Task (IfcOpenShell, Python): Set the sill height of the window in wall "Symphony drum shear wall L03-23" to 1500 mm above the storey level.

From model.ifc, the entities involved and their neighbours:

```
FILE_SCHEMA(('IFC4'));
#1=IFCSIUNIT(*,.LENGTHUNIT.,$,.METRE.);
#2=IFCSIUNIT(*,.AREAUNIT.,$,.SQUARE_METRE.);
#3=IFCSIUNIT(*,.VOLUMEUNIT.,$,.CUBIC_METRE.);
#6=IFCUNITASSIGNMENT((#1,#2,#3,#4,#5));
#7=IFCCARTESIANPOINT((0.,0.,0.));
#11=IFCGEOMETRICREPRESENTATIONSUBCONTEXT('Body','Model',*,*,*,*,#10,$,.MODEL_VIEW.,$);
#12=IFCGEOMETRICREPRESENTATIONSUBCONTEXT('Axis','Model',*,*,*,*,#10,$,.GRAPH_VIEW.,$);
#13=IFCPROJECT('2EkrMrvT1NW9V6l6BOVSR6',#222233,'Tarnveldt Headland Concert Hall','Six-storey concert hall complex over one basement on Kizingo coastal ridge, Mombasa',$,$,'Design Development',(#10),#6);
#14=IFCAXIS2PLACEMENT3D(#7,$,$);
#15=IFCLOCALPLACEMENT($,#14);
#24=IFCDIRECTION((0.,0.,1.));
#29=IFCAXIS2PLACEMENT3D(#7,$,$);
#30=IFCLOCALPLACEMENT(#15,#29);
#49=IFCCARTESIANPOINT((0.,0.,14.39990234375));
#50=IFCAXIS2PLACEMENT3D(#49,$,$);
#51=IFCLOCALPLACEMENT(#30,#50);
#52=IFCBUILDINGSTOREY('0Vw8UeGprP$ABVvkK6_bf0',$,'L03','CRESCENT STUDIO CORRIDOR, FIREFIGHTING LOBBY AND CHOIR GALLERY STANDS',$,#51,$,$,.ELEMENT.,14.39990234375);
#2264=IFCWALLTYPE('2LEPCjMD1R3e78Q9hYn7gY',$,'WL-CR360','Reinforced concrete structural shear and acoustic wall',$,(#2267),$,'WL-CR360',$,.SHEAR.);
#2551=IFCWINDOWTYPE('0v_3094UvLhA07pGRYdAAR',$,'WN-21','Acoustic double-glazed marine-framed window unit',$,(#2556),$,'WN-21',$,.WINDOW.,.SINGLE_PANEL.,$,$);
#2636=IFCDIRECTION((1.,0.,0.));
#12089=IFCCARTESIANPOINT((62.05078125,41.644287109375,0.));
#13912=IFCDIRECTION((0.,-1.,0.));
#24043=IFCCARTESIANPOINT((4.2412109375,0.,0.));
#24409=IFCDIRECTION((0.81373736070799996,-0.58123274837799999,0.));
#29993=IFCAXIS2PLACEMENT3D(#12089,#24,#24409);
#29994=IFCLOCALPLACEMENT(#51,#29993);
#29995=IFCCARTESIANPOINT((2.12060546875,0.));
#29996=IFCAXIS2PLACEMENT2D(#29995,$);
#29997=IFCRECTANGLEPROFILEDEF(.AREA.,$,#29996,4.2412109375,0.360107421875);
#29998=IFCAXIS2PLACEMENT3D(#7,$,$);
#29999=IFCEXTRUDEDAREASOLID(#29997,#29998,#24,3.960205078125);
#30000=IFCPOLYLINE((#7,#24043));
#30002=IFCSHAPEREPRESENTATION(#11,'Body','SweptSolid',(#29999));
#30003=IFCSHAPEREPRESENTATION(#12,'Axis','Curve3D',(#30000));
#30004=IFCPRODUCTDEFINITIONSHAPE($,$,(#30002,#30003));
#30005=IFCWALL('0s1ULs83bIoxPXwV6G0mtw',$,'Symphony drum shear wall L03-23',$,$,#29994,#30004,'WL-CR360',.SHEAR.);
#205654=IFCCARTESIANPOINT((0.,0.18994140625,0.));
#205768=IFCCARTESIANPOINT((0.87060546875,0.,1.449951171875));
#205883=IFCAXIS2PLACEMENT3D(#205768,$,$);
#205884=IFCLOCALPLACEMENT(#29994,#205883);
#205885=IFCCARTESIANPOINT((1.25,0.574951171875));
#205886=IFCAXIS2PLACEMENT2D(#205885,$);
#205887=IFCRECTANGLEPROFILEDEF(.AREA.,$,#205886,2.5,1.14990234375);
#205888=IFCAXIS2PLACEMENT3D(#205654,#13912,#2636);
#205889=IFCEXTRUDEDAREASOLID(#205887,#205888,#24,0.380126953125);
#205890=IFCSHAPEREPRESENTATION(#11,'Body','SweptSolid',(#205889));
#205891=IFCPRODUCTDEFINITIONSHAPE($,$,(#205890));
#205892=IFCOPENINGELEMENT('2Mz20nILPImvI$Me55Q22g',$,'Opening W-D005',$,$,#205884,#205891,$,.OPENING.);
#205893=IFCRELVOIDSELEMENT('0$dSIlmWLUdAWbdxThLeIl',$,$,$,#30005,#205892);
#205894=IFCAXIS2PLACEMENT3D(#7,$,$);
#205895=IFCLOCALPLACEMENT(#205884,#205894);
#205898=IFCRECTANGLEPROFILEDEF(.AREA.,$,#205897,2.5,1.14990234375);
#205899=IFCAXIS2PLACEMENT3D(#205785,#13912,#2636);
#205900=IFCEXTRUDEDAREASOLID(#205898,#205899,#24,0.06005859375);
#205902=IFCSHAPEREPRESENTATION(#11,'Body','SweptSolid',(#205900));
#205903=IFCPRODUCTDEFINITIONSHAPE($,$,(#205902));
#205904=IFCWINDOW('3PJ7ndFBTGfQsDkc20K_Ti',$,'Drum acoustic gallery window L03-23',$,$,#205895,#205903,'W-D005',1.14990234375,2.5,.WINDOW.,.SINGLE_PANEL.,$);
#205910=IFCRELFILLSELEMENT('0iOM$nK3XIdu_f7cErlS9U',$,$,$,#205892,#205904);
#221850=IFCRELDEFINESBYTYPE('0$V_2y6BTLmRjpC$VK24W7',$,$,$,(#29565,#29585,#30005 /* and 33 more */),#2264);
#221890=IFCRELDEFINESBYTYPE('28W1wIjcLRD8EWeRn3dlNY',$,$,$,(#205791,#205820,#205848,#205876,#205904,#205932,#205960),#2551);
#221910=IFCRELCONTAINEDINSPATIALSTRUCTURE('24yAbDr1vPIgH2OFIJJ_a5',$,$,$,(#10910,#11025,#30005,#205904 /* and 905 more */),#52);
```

```python
import numpy as np
import ifcopenshell
import ifcopenshell.api.geometry
import ifcopenshell.geom
import ifcopenshell.util.element
import ifcopenshell.util.placement
import ifcopenshell.util.shape
import ifcopenshell.util.unit

model = ifcopenshell.open("model.ifc")
unit_scale = ifcopenshell.util.unit.calculate_unit_scale(model)

window = model.by_guid("3PJ7ndFBTGfQsDkc20K_Ti")
opening = window.FillsVoids[0].RelatingOpeningElement
storey = ifcopenshell.util.element.get_container(window, ifc_class="IfcBuildingStorey")
level = ifcopenshell.util.placement.get_local_placement(storey.ObjectPlacement)[2, 3]

# The opening's origin need not be at the sill, so measure its lowest point.
shape = ifcopenshell.geom.create_shape(ifcopenshell.geom.settings(), opening)
bottom = ifcopenshell.util.shape.get_shape_bottom_elevation(shape, shape.geometry) / unit_scale
dz = level + 1.5 - bottom

shift = np.array([0.0, 0.0, dz])
# The window is placed relative to its opening, so it follows when the opening moves.
matrix = ifcopenshell.util.placement.get_local_placement(opening.ObjectPlacement)
matrix[:3, 3] += shift
ifcopenshell.api.geometry.edit_object_placement(
    model, product=opening, matrix=matrix, is_si=False, should_transform_children=True
)

print(f"moved by {dz * unit_scale:+.3f} m")

model.write("model_updated.ifc")
```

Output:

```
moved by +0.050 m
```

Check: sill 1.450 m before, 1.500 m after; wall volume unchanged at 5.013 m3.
